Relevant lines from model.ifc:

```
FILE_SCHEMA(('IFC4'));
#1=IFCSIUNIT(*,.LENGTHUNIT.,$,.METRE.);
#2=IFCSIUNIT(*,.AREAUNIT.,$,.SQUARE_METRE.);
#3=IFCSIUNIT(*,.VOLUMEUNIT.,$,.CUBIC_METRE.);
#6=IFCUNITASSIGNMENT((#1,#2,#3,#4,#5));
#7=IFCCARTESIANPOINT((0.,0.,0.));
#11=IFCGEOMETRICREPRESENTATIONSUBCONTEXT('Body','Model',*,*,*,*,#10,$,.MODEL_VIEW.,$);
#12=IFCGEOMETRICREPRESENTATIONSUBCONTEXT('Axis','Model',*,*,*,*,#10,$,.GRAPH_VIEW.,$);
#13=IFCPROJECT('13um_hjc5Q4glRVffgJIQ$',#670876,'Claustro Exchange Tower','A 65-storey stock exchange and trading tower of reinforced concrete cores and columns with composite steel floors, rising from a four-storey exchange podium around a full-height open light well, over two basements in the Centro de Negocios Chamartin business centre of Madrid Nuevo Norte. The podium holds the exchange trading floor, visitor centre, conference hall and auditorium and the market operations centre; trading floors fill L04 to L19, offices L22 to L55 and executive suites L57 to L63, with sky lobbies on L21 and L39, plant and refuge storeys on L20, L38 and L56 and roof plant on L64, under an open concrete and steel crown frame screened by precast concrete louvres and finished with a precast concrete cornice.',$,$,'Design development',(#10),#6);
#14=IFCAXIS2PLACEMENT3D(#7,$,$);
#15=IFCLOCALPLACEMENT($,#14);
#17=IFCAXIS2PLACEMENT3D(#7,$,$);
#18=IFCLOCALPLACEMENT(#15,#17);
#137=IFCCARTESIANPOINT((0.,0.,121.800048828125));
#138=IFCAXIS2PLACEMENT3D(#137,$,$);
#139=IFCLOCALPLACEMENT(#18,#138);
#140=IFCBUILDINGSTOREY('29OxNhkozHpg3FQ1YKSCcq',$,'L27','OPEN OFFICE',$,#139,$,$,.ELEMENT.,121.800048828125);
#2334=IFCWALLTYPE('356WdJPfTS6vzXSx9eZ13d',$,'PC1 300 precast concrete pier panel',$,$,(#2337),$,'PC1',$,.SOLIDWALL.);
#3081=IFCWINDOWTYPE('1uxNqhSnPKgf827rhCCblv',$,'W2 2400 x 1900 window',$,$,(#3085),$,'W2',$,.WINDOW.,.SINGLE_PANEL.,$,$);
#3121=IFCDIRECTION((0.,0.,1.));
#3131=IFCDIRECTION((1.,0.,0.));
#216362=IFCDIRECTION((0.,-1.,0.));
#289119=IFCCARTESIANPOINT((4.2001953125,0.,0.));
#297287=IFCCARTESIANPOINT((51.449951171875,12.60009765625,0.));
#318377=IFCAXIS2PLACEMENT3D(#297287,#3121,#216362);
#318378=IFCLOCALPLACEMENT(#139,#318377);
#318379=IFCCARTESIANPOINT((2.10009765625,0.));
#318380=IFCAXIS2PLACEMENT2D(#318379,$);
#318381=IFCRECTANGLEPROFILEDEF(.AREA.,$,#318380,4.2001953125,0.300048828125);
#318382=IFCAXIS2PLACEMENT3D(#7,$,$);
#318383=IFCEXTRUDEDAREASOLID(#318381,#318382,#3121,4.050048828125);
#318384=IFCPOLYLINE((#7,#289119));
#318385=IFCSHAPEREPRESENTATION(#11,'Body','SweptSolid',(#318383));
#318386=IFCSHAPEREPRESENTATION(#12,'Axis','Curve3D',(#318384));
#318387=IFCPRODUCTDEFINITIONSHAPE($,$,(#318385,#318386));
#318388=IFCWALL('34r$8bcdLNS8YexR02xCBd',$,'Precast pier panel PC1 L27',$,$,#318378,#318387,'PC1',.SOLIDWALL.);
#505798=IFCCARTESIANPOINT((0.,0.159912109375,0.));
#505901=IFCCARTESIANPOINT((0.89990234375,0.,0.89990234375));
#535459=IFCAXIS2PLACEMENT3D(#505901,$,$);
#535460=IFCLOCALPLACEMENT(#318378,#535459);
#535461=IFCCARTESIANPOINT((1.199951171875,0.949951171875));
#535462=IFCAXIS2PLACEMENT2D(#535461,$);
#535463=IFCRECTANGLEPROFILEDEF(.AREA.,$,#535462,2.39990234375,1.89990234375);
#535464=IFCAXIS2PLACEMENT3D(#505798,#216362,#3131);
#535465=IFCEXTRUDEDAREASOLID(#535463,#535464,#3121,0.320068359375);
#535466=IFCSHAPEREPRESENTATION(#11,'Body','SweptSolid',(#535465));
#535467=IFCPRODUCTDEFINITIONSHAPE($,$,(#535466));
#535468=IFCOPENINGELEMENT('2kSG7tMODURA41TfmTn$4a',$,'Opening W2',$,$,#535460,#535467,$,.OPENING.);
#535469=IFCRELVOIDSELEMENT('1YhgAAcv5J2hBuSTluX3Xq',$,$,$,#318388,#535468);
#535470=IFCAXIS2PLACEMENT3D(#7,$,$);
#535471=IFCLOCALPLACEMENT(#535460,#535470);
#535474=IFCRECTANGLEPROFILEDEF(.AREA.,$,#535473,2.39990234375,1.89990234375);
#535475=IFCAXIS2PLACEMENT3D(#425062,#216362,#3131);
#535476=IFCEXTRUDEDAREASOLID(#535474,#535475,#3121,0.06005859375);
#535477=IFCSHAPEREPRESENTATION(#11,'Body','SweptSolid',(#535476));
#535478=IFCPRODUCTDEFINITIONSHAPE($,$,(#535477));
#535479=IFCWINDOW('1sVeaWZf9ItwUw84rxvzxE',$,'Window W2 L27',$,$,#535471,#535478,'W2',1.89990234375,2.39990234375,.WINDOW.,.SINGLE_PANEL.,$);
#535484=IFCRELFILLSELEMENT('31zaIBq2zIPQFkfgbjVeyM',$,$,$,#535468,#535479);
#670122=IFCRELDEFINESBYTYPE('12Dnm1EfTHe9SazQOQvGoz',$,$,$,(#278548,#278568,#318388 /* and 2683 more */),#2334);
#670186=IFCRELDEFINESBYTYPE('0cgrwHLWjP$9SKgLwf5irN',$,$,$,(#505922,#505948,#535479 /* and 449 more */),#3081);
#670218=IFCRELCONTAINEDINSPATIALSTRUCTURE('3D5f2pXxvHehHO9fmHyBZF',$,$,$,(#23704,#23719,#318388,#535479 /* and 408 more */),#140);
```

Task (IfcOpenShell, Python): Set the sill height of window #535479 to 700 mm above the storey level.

```python
import numpy as np
import ifcopenshell
import ifcopenshell.api.geometry
import ifcopenshell.geom
import ifcopenshell.util.element
import ifcopenshell.util.placement
import ifcopenshell.util.shape
import ifcopenshell.util.unit

model = ifcopenshell.open("model.ifc")
unit_scale = ifcopenshell.util.unit.calculate_unit_scale(model)

window = model.by_guid("1sVeaWZf9ItwUw84rxvzxE")
opening = window.FillsVoids[0].RelatingOpeningElement
storey = ifcopenshell.util.element.get_container(window, ifc_class="IfcBuildingStorey")
level = ifcopenshell.util.placement.get_local_placement(storey.ObjectPlacement)[2, 3]

# The opening's origin need not be at the sill, so measure its lowest point.
shape = ifcopenshell.geom.create_shape(ifcopenshell.geom.settings(), opening)
bottom = ifcopenshell.util.shape.get_shape_bottom_elevation(shape, shape.geometry) / unit_scale
dz = level + 0.7 / unit_scale - bottom

shift = np.array([0.0, 0.0, dz])
# The window is placed relative to its opening, so it follows when the opening moves.
matrix = ifcopenshell.util.placement.get_local_placement(opening.ObjectPlacement)
matrix[:3, 3] += shift
ifcopenshell.api.geometry.edit_object_placement(
    model, product=opening, matrix=matrix, is_si=False, should_transform_children=True
)

print(f"moved by {dz * unit_scale:+.3f} m")

model.write("model-out.ifc")
```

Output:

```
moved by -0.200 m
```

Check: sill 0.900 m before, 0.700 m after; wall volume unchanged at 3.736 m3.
